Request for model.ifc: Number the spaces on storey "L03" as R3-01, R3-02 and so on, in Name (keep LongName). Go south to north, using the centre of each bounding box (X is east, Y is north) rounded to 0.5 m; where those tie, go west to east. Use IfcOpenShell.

First a look at what the model holds.

```python
import ifcopenshell
import ifcopenshell.util.element
import ifcopenshell.util.placement

model = ifcopenshell.open("model.ifc")
print(model.schema)
storey = next(s for s in model.by_type("IfcBuildingStorey") if s.Name == "L03")
spaces = [e for e in ifcopenshell.util.element.get_decomposition(storey) if e.is_a("IfcSpace")]
for e in sorted(spaces, key=lambda e: e.id()):
    origin = ifcopenshell.util.placement.get_local_placement(e.ObjectPlacement)[:3, 3]
    print(e.id(), e.Name, e.LongName, origin.round(2) + 0.0, sep=" | ")
```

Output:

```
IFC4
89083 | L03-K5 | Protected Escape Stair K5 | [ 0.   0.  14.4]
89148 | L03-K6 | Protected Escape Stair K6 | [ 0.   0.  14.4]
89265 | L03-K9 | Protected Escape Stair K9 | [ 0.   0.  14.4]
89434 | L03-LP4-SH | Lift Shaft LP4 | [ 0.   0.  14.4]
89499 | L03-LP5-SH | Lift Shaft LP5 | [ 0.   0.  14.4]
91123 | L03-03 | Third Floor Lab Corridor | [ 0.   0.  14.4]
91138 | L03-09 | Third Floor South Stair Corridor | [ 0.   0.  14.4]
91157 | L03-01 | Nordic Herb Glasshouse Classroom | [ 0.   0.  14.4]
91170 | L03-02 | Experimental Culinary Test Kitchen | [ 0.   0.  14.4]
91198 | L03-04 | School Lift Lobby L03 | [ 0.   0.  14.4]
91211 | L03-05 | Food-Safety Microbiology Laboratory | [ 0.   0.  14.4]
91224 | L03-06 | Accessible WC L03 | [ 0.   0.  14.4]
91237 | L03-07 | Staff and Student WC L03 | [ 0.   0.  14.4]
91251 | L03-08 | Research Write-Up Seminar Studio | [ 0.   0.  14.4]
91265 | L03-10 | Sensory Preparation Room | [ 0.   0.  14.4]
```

```python
import ifcopenshell
import ifcopenshell.geom
import ifcopenshell.util.element
import ifcopenshell.util.shape

model = ifcopenshell.open("model.ifc")
settings = ifcopenshell.geom.settings()
settings.set("use-world-coords", True)


def centre(element):
    shape = ifcopenshell.geom.create_shape(settings, element)
    return ifcopenshell.util.shape.get_bbox_centroid(shape.geometry)


storey = next(s for s in model.by_type("IfcBuildingStorey") if s.Name == "L03")
spaces = [e for e in ifcopenshell.util.element.get_decomposition(storey) if e.is_a("IfcSpace")]

# Insertion points can sit at a corner or the storey origin, so sort by the geometry (in metres).
centres = {e: centre(e) for e in spaces}
spaces.sort(key=lambda e: (round(centres[e][1] / 0.5), centres[e][0]))

for i, e in enumerate(spaces, start=1):
    number = f"R3-{i:02d}"
    e.Name = number
    print(e.id(), number)

model.write("model_edited.ifc")
```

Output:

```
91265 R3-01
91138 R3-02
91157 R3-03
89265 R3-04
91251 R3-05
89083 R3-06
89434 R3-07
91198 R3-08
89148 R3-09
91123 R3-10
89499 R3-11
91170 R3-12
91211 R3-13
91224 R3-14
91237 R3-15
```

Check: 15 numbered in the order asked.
